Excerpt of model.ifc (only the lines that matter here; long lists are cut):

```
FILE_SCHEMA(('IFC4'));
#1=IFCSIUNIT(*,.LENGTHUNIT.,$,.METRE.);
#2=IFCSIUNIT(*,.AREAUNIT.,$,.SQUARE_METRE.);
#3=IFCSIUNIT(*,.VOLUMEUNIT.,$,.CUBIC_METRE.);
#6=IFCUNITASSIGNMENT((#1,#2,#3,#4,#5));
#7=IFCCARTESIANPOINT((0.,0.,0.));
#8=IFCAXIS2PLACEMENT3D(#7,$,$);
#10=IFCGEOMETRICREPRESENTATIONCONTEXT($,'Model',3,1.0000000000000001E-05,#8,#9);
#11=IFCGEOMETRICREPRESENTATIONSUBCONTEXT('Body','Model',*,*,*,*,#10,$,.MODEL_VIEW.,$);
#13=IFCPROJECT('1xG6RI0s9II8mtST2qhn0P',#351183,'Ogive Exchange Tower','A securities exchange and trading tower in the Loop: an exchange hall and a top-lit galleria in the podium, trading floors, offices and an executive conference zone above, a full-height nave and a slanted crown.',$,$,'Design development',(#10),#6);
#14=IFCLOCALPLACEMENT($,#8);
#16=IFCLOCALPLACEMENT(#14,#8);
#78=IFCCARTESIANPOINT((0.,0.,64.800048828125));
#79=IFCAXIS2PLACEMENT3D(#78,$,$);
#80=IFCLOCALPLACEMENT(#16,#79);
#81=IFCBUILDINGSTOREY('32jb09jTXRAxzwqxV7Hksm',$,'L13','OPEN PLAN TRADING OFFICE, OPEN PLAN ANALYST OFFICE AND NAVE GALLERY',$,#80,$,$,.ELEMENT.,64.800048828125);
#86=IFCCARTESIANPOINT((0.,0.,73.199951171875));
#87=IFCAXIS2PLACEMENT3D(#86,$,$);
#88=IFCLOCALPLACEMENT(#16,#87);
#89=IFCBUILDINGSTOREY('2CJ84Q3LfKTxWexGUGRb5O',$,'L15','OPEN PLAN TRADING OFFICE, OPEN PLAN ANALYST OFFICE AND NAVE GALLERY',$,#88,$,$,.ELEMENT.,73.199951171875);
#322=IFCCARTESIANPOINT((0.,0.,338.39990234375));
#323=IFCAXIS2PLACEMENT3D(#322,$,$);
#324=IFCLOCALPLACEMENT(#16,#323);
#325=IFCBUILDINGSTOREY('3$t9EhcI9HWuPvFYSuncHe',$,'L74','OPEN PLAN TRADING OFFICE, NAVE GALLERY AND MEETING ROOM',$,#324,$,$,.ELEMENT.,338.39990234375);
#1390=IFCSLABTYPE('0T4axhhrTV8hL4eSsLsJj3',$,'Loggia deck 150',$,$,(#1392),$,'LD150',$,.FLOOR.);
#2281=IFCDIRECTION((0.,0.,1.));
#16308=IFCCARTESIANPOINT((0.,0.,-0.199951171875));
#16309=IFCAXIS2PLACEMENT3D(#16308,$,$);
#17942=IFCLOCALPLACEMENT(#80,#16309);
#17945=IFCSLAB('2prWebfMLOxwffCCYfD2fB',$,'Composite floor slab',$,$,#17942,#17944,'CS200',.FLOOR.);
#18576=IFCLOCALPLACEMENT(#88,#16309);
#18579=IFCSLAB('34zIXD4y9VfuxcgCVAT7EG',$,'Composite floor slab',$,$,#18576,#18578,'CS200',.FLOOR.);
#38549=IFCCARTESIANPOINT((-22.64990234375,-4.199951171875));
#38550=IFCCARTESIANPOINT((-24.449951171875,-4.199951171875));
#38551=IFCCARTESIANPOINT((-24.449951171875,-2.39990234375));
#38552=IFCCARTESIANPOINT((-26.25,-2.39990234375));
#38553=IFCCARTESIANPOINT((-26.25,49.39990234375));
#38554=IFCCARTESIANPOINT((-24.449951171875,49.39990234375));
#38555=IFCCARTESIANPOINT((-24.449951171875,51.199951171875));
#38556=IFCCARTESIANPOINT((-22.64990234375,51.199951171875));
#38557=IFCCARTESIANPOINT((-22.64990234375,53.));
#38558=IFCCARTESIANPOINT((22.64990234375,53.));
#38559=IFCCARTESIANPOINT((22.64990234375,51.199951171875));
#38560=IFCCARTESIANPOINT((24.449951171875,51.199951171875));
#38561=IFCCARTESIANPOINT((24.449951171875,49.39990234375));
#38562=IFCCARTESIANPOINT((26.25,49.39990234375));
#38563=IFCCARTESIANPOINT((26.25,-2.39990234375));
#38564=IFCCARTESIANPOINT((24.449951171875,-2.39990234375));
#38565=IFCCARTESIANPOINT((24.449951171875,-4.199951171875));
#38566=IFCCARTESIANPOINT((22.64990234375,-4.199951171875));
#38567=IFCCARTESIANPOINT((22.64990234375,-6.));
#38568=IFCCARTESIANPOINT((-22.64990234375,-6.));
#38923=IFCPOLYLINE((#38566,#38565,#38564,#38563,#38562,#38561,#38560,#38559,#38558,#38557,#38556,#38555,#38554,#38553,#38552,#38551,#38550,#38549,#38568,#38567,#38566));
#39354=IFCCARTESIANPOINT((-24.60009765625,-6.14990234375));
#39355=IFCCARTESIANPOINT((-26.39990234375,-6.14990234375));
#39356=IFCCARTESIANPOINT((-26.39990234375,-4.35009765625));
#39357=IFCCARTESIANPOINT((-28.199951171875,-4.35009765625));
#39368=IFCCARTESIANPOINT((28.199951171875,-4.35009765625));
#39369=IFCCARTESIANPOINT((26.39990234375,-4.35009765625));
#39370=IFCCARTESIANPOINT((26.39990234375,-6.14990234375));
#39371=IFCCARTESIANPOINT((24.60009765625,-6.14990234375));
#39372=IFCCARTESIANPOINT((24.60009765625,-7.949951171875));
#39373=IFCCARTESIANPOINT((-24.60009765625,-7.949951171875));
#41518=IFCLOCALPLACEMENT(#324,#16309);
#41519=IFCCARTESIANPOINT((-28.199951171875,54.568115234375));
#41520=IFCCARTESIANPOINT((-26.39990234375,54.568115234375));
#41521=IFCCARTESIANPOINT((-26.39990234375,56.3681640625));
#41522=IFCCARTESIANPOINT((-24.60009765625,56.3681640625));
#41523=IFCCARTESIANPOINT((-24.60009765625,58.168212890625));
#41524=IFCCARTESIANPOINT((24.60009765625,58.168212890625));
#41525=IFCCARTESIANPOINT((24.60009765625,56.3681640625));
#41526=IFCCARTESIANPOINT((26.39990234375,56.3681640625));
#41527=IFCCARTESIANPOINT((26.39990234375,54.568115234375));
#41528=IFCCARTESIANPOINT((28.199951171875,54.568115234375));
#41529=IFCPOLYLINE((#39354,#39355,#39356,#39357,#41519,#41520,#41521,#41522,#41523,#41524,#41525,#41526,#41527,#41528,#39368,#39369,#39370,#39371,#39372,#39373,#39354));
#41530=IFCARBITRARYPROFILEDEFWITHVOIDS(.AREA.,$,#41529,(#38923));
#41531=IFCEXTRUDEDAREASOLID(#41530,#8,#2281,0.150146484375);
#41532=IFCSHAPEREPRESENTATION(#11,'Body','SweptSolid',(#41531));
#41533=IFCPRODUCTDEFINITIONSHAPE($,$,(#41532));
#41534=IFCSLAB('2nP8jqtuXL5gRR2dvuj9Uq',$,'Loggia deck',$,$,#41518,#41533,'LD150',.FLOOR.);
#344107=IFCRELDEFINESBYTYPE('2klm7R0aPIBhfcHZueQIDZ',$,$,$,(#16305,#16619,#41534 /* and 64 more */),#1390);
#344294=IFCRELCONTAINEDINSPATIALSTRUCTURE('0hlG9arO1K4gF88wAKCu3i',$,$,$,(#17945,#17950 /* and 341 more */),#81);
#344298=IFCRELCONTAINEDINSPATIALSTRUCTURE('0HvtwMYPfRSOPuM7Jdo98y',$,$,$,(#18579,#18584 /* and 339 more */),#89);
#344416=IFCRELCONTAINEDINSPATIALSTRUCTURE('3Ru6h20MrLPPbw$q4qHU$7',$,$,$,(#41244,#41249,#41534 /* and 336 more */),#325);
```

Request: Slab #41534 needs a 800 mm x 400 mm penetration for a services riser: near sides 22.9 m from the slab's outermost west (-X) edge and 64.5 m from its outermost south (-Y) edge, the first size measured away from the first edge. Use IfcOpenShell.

```python
import numpy as np
import ifcopenshell
import ifcopenshell.api.feature
import ifcopenshell.api.geometry
import ifcopenshell.api.root
import ifcopenshell.geom
import ifcopenshell.util.placement
import ifcopenshell.util.representation
import ifcopenshell.util.shape
import ifcopenshell.util.unit

model = ifcopenshell.open("model.ifc")
unit_scale = ifcopenshell.util.unit.calculate_unit_scale(model)
settings = ifcopenshell.geom.settings()


def volume(element):
    """Net volume in cubic metres, openings subtracted."""
    shape = ifcopenshell.geom.create_shape(settings, element)
    return ifcopenshell.util.shape.get_volume(shape.geometry)


slab = model.by_guid("2nP8jqtuXL5gRR2dvuj9Uq")
before = volume(slab)

# Extent in the slab's own axes, in metres. The edges named are its -X and -Y sides.
slab_shape = ifcopenshell.geom.create_shape(settings, slab)
vertices = ifcopenshell.util.shape.get_vertices(slab_shape.geometry)
x_min, y_min, bottom = vertices.min(axis=0)
top = vertices[:, 2].max()

opening = ifcopenshell.api.root.create_entity(model, ifc_class="IfcOpeningElement", name="Services riser opening", predefined_type="OPENING")
context = ifcopenshell.util.representation.get_context(model, "Model", "Body", "MODEL_VIEW")
width, depth = 0.8, 0.4
outline = [(0.0, 0.0), (width, 0.0), (width, depth), (0.0, depth), (0.0, 0.0)]
# Overshoot both faces by 50 mm so the cut is clean.
shape = ifcopenshell.api.geometry.add_slab_representation(
    model, context=context, depth=top - bottom + 0.1, polyline=outline
)
ifcopenshell.api.geometry.assign_representation(model, product=opening, representation=shape)

matrix = ifcopenshell.util.placement.get_local_placement(slab.ObjectPlacement)
matrix[:, 3] = matrix @ np.append(np.array([x_min + 22.9, y_min + 64.5, bottom - 0.05]) / unit_scale, 1.0)
ifcopenshell.api.geometry.edit_object_placement(model, product=opening, matrix=matrix, is_si=False)
ifcopenshell.api.feature.add_feature(model, feature=opening, element=slab)

after = volume(slab)

print(f"slab volume {before:.3f} -> {after:.3f} m3")

model.write("model_updated.ifc")
```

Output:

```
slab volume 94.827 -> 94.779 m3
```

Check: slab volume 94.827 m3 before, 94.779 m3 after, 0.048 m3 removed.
